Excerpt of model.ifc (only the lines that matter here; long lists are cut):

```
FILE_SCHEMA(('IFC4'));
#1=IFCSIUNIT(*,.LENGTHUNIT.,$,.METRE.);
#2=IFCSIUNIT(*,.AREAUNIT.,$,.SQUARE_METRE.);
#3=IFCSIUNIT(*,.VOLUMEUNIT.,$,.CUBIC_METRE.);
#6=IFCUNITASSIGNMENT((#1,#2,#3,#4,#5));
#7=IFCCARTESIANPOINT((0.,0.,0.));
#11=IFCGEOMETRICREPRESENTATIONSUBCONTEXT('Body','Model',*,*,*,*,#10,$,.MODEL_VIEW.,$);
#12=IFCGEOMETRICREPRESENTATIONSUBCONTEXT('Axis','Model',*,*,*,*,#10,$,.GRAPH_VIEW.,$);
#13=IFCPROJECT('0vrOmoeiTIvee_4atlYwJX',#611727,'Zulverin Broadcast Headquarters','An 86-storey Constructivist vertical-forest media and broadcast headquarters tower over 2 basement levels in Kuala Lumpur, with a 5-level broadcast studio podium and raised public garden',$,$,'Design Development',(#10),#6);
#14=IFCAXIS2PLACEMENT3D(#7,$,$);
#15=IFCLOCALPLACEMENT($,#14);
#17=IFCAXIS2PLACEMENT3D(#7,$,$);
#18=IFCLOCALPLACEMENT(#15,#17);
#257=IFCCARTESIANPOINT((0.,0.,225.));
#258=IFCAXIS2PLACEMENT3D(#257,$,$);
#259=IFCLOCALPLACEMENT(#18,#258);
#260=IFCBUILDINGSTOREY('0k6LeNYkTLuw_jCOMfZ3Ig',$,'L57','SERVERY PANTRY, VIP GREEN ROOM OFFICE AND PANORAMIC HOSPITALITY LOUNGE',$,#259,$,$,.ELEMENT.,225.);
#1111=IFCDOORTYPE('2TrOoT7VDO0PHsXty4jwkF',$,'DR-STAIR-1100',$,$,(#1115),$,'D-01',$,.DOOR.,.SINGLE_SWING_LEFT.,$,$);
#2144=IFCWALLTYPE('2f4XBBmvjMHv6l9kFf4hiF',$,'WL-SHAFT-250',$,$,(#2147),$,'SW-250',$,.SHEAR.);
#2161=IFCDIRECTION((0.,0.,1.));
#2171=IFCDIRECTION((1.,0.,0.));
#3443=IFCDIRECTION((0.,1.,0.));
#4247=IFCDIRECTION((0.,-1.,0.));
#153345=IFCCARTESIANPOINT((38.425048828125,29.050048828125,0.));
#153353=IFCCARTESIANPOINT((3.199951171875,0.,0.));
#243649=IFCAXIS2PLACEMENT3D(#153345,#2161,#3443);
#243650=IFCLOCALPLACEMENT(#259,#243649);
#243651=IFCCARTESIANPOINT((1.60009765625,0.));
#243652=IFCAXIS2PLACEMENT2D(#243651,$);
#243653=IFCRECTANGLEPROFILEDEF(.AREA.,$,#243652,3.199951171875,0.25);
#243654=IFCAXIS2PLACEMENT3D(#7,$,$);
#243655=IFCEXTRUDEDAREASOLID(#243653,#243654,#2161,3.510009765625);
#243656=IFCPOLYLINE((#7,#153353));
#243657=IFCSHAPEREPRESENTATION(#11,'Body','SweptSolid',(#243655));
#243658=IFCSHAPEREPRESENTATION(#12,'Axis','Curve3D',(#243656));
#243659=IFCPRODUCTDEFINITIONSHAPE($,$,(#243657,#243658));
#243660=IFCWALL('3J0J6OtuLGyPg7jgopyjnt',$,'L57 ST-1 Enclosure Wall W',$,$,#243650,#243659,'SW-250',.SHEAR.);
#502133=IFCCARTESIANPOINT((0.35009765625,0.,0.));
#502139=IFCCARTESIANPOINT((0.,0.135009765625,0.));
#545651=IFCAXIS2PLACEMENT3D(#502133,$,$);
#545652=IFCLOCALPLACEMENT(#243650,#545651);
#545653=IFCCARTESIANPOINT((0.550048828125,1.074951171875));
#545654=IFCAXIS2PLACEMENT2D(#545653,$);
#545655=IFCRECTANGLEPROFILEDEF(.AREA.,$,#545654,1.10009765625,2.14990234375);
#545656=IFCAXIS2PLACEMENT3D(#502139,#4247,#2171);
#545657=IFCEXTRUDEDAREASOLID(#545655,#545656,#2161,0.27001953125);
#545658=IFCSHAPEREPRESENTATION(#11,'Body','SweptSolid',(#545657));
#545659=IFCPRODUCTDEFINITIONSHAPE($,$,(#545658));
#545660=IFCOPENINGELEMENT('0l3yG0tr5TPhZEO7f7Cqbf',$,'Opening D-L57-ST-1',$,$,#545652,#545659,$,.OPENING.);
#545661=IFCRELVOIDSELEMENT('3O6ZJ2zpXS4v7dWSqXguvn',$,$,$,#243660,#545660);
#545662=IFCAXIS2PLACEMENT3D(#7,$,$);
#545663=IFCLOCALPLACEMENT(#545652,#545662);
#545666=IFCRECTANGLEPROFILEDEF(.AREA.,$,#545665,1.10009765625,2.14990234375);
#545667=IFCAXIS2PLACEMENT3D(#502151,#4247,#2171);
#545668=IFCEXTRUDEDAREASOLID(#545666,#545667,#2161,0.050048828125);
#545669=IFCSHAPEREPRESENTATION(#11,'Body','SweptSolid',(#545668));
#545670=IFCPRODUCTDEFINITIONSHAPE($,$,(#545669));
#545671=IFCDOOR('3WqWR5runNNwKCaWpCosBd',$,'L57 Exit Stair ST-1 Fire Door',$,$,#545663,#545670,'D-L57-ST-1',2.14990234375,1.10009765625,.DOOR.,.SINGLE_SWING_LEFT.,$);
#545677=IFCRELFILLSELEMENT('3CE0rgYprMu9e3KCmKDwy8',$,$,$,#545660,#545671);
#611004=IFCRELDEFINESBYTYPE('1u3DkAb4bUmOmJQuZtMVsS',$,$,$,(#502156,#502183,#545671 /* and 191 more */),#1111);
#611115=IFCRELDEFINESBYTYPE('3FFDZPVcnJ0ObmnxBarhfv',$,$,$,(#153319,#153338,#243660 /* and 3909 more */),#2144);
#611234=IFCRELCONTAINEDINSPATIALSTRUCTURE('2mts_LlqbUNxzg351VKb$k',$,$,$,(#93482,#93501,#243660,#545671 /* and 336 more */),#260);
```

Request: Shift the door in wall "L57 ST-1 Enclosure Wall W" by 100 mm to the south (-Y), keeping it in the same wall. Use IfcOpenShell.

```python
import ifcopenshell
import ifcopenshell.api.geometry
import ifcopenshell.util.placement

model = ifcopenshell.open("model.ifc")

door = model.by_guid("3WqWR5runNNwKCaWpCosBd")
opening = door.FillsVoids[0].RelatingOpeningElement
wall = opening.VoidsElements[0].RelatingBuildingElement

wall_matrix = ifcopenshell.util.placement.get_local_placement(wall.ObjectPlacement)
shift = wall_matrix[:3, 0] * -0.1
before = ifcopenshell.util.placement.get_local_placement(door.ObjectPlacement)[:3, 3].copy()

# The door is placed relative to its opening, so it follows when the opening moves.
matrix = ifcopenshell.util.placement.get_local_placement(opening.ObjectPlacement)
matrix[:3, 3] += shift
ifcopenshell.api.geometry.edit_object_placement(
    model, product=opening, matrix=matrix, is_si=False, should_transform_children=True
)

after = ifcopenshell.util.placement.get_local_placement(door.ObjectPlacement)[:3, 3]
print("door moved by", (after - before).round(3) + 0.0)

model.write("model_v2.ifc")
```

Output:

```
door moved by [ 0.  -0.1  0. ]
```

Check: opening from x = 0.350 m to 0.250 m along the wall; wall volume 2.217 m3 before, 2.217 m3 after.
